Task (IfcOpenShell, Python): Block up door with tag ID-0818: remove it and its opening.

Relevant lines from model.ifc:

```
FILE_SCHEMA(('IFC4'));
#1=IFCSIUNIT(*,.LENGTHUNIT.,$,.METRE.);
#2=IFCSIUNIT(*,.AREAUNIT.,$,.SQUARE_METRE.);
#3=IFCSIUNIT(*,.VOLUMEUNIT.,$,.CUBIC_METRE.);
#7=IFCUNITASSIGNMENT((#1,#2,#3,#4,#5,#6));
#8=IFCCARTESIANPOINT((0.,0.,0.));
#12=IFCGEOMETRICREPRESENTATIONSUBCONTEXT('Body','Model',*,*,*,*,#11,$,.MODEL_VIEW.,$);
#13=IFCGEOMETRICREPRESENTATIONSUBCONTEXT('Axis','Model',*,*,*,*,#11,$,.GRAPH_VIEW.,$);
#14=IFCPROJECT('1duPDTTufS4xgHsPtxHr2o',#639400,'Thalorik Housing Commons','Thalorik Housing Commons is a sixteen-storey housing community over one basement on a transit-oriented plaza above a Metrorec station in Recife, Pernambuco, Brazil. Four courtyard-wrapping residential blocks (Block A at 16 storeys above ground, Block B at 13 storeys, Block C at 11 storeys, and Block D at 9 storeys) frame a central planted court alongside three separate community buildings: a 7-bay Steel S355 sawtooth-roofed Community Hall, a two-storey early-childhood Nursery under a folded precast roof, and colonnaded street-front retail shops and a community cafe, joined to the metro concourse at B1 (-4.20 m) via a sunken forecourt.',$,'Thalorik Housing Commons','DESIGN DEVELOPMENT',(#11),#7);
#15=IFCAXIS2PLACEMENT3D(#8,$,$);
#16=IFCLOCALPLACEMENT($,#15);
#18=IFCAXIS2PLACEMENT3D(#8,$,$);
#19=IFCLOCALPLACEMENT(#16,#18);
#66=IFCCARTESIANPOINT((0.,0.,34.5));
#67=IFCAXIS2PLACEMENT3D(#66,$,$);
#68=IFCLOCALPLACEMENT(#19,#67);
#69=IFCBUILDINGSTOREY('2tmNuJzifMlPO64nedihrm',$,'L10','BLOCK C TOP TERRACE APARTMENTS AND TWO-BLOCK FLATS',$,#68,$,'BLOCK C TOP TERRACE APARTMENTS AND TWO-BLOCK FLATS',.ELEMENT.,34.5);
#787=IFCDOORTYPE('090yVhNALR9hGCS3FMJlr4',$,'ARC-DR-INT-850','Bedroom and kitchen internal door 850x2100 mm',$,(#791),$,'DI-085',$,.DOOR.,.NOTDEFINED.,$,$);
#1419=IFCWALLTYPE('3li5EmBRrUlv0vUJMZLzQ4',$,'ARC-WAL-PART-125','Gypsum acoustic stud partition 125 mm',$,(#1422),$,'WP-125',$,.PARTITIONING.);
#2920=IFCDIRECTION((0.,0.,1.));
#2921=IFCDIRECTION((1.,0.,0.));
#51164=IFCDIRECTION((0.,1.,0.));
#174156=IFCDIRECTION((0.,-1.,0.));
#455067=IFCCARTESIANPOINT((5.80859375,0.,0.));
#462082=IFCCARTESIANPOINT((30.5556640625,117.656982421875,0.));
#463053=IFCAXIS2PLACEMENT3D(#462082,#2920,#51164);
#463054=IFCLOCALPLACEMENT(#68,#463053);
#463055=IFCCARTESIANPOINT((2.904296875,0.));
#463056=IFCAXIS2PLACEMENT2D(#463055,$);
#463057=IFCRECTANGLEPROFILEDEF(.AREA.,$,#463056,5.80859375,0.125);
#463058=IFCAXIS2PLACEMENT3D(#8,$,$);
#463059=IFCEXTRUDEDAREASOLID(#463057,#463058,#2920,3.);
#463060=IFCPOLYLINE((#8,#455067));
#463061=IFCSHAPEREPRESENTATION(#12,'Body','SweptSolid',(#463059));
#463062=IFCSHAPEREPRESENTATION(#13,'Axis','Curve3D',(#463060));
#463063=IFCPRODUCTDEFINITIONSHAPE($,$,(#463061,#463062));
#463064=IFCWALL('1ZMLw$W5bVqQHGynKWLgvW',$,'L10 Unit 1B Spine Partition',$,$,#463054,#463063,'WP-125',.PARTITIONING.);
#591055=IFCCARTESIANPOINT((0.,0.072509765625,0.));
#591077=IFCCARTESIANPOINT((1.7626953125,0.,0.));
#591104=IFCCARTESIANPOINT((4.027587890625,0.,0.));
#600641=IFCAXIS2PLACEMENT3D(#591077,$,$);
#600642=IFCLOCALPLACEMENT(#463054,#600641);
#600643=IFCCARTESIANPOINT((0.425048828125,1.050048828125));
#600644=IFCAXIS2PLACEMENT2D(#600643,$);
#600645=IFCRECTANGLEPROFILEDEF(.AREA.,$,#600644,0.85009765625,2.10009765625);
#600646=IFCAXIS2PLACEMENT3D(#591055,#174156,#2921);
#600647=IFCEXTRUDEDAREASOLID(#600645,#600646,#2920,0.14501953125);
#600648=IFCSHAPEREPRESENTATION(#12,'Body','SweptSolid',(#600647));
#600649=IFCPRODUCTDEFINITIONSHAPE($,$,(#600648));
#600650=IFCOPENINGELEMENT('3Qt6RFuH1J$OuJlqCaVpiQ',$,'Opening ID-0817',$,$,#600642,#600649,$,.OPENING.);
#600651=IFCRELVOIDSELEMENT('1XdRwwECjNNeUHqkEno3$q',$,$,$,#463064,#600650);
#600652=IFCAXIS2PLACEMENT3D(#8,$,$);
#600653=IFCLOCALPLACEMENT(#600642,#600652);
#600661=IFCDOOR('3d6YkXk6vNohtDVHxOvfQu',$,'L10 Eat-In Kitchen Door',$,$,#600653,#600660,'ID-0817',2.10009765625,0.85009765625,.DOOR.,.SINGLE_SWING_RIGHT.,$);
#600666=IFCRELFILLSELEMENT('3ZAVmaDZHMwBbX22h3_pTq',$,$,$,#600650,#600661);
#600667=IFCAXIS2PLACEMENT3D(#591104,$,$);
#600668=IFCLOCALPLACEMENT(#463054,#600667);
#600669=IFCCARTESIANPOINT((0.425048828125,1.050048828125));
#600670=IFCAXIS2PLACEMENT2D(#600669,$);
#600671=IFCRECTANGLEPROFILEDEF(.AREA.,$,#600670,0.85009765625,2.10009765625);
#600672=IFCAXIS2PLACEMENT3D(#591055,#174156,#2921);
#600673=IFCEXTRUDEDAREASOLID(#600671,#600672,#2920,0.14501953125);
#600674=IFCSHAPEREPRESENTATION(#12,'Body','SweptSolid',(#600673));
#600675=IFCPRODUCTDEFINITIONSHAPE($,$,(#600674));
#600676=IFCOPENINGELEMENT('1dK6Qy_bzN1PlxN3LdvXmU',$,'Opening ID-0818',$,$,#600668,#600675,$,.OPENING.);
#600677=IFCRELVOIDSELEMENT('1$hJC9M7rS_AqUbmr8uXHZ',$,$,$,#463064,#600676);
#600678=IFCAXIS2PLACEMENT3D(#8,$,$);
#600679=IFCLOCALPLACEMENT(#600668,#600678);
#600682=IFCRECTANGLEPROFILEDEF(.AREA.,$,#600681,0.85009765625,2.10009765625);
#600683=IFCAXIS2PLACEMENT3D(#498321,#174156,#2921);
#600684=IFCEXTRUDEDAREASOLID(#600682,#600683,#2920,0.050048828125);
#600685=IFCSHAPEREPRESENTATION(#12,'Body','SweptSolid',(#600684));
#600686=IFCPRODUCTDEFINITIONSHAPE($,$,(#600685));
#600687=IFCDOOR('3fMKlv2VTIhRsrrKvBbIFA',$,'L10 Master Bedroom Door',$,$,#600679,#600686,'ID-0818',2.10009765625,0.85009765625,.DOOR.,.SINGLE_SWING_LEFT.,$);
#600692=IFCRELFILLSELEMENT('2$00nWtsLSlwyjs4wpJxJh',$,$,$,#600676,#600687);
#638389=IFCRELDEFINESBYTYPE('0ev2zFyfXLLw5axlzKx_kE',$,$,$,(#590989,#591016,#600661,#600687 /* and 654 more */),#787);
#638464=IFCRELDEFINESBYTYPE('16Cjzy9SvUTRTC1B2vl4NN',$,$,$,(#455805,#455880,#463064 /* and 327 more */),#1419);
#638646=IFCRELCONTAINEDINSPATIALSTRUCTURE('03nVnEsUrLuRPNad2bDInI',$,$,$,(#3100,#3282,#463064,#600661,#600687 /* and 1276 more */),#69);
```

```python
import ifcopenshell
import ifcopenshell.api.feature
import ifcopenshell.api.root
import ifcopenshell.geom
import ifcopenshell.util.shape

model = ifcopenshell.open("model.ifc")
settings = ifcopenshell.geom.settings()


def volume(element):
    """Net volume in cubic metres, openings subtracted."""
    shape = ifcopenshell.geom.create_shape(settings, element)
    return ifcopenshell.util.shape.get_volume(shape.geometry)


door = model.by_guid("3fMKlv2VTIhRsrrKvBbIFA")
opening = door.FillsVoids[0].RelatingOpeningElement
wall = opening.VoidsElements[0].RelatingBuildingElement
before = volume(wall)

ifcopenshell.api.root.remove_product(model, product=door)
ifcopenshell.api.feature.remove_feature(model, feature=opening)

after = volume(wall)

print(f"wall volume {before:.3f} -> {after:.3f} m3")

model.write("model_v2.ifc")
```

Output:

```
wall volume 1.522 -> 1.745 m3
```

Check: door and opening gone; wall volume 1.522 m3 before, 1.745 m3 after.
